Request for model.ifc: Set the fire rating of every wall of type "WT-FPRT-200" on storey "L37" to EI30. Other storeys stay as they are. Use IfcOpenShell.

First a look at what the model holds.

```python
import ifcopenshell
import ifcopenshell.util.element

model = ifcopenshell.open("model.ifc")
print(model.schema)
storey = next(s for s in model.by_type("IfcBuildingStorey") if s.Name == "L37")
walls = [e for e in ifcopenshell.util.element.get_decomposition(storey) if e.is_a("IfcWall")]
seen = {}
for e in walls:
    element_type = ifcopenshell.util.element.get_type(e)
    key = (element_type.Name if element_type != e and element_type else None, ifcopenshell.util.element.get_pset(e, "Pset_WallCommon", "FireRating"))
    seen[key] = seen.get(key, 0) + 1
for (name, value), count in sorted(seen.items(), key=str):
    print(count, "x", name, "|", value)
```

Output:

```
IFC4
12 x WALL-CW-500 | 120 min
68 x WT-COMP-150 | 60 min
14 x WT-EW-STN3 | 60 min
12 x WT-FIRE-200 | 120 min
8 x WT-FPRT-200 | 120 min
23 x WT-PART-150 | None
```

```python
import ifcopenshell
import ifcopenshell.api.pset
import ifcopenshell.util.element

model = ifcopenshell.open("model.ifc")

storey = next(s for s in model.by_type("IfcBuildingStorey") if s.Name == "L37")
walls = [e for e in ifcopenshell.util.element.get_decomposition(storey) if e.is_a("IfcWall")]

count = 0
for e in walls:
    element_type = ifcopenshell.util.element.get_type(e)
    if element_type in (None, e) or element_type.Name != "WT-FPRT-200":
        continue
    found = ifcopenshell.util.element.get_pset(e, "Pset_WallCommon", should_inherit=False)
    if found:
        pset = model.by_id(found["id"])
        if len(ifcopenshell.util.element.get_elements_by_pset(pset)) > 1:
            pset = ifcopenshell.api.pset.unshare_pset(model, products=[e], pset=pset)[0]
    else:
        pset = ifcopenshell.api.pset.add_pset(model, product=e, name="Pset_WallCommon")
    ifcopenshell.api.pset.edit_pset(model, pset=pset, properties={"FireRating": "EI30"})
    count += 1

print(count, "walls updated")

model.write("model-out.ifc")
```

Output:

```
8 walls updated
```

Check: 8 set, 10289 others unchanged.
